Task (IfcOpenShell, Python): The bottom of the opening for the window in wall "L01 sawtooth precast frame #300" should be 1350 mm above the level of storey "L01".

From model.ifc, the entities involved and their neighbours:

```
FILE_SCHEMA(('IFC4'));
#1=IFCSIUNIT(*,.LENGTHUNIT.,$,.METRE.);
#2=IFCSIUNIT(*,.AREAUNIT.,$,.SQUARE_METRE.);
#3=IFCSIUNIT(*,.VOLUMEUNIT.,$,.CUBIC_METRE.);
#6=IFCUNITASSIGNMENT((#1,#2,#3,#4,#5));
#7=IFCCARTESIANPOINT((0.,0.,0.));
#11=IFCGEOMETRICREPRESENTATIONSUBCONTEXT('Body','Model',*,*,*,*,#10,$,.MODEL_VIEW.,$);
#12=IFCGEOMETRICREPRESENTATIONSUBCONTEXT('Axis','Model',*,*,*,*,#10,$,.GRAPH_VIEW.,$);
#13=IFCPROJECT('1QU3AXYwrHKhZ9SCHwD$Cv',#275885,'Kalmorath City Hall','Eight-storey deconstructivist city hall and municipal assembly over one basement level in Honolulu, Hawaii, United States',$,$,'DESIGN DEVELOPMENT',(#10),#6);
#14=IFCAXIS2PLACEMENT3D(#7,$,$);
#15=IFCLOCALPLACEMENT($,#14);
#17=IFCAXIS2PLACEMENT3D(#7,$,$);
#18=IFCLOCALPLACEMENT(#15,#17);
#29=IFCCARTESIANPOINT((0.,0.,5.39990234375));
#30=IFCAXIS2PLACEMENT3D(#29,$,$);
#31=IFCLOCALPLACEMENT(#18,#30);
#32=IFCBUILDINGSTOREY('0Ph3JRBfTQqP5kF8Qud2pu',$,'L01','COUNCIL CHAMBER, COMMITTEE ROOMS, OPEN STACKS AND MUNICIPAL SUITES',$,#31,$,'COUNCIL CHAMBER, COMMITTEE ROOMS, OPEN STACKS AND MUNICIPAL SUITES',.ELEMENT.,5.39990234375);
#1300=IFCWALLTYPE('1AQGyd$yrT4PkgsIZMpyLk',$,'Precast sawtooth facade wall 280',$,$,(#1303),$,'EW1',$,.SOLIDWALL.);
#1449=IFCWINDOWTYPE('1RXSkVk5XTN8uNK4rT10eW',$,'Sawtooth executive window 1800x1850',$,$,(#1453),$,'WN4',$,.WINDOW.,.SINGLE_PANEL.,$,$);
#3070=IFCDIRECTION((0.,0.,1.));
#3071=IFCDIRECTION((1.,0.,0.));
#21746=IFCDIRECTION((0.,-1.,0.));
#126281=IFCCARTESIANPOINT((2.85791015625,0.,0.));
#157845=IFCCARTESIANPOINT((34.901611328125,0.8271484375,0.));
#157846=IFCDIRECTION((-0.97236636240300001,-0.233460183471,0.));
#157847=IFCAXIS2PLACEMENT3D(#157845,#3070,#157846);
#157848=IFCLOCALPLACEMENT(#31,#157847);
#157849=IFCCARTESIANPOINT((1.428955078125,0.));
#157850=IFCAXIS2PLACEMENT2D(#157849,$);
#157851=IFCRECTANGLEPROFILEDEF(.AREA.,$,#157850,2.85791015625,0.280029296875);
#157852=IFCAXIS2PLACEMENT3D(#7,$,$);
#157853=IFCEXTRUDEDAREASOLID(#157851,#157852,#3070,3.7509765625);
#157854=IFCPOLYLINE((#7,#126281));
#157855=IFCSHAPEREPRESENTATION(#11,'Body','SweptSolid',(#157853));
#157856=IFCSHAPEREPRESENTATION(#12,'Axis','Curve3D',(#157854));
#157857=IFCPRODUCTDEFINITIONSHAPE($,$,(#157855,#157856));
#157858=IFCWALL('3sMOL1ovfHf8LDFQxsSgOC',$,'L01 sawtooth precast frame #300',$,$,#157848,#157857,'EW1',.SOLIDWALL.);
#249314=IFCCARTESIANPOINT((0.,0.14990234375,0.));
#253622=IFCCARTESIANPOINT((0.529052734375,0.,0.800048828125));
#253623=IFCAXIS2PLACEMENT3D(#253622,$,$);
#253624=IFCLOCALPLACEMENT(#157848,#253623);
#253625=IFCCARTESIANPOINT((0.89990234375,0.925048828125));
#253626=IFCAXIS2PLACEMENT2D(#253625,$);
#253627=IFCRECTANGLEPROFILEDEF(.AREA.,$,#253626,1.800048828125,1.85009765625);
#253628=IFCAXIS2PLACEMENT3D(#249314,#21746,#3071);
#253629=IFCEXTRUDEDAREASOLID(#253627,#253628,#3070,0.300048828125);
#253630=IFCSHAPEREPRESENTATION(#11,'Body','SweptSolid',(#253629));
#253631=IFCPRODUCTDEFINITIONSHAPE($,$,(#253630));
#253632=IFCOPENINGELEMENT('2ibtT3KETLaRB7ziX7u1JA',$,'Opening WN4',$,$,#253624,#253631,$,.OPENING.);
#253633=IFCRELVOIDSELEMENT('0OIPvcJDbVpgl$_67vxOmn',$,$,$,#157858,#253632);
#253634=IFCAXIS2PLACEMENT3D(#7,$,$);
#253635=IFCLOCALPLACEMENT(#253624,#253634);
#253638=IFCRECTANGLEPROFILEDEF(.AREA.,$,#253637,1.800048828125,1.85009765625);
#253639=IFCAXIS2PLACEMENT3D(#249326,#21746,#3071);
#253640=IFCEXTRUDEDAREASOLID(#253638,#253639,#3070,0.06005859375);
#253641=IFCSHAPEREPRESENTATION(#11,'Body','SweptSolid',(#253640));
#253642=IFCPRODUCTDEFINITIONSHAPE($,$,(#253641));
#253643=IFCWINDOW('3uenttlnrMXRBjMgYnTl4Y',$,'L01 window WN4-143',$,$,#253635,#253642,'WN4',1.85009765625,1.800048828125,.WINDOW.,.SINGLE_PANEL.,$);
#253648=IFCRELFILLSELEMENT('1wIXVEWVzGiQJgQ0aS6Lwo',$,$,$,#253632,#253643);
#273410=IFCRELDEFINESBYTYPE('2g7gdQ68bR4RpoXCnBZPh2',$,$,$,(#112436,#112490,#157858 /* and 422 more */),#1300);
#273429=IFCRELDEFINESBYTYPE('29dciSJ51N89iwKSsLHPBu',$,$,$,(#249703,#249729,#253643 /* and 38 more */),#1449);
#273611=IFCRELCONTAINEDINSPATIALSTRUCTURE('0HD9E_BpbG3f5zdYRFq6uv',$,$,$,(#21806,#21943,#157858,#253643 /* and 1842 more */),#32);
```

```python
import numpy as np
import ifcopenshell
import ifcopenshell.api.geometry
import ifcopenshell.geom
import ifcopenshell.util.element
import ifcopenshell.util.placement
import ifcopenshell.util.shape
import ifcopenshell.util.unit

model = ifcopenshell.open("model.ifc")
unit_scale = ifcopenshell.util.unit.calculate_unit_scale(model)

window = model.by_guid("3uenttlnrMXRBjMgYnTl4Y")
opening = window.FillsVoids[0].RelatingOpeningElement
storey = ifcopenshell.util.element.get_container(window, ifc_class="IfcBuildingStorey")
level = ifcopenshell.util.placement.get_local_placement(storey.ObjectPlacement)[2, 3]

# The opening's origin need not be at the sill, so measure its lowest point.
shape = ifcopenshell.geom.create_shape(ifcopenshell.geom.settings(), opening)
bottom = ifcopenshell.util.shape.get_shape_bottom_elevation(shape, shape.geometry) / unit_scale
dz = level + 1.35 / unit_scale - bottom

shift = np.array([0.0, 0.0, dz])
# The window is placed relative to its opening, so it follows when the opening moves.
matrix = ifcopenshell.util.placement.get_local_placement(opening.ObjectPlacement)
matrix[:3, 3] += shift
ifcopenshell.api.geometry.edit_object_placement(
    model, product=opening, matrix=matrix, is_si=False, should_transform_children=True
)

print(f"moved by {dz * unit_scale:+.3f} m")

model.write("model_updated.ifc")
```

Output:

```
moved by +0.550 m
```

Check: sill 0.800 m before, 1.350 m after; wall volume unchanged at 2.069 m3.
